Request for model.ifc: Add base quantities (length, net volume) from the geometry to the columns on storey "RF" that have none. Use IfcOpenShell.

First a look at what the model holds.

```python
import ifcopenshell
import ifcopenshell.util.element
import ifcopenshell.util.unit

model = ifcopenshell.open("model.ifc")
print(model.schema)
for unit_type in ("LENGTHUNIT", "AREAUNIT", "VOLUMEUNIT"):
    print(unit_type, ifcopenshell.util.unit.calculate_unit_scale(model, unit_type))
storey = next(s for s in model.by_type("IfcBuildingStorey") if s.Name == "RF")
columns = [e for e in ifcopenshell.util.element.get_decomposition(storey) if e.is_a("IfcColumn")]
for e in sorted(columns, key=lambda e: e.id()):
    print(e.id(), e.is_a(), e.Name, list(ifcopenshell.util.element.get_psets(e, qtos_only=True)), sep=" | ")
```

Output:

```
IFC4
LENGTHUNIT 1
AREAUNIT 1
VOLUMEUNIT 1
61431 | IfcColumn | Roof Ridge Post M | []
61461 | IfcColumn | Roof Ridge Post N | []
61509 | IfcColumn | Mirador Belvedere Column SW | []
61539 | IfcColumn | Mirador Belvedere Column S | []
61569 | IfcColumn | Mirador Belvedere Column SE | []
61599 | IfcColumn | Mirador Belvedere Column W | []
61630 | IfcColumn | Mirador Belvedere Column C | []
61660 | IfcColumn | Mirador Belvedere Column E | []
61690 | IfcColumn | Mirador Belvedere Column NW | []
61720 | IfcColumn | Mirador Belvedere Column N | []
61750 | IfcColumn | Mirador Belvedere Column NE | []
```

```python
import ifcopenshell
import ifcopenshell.api.pset
import ifcopenshell.geom
import ifcopenshell.util.element
import ifcopenshell.util.shape
import ifcopenshell.util.unit

model = ifcopenshell.open("model.ifc")
unit_scale = ifcopenshell.util.unit.calculate_unit_scale(model)
volume_scale = ifcopenshell.util.unit.calculate_unit_scale(model, "VOLUMEUNIT")
settings = ifcopenshell.geom.settings()

storey = next(s for s in model.by_type("IfcBuildingStorey") if s.Name == "RF")
columns = [e for e in ifcopenshell.util.element.get_decomposition(storey) if e.is_a("IfcColumn")]

for e in sorted(columns, key=lambda e: e.id()):
    if ifcopenshell.util.element.get_psets(e, qtos_only=True, should_inherit=False):
        continue
    # Geometry comes back in metres, in the element's own axes.
    shape = ifcopenshell.geom.create_shape(settings, e)
    values = {
        "Length": ifcopenshell.util.shape.get_z(shape.geometry) / unit_scale,
        "NetVolume": ifcopenshell.util.shape.get_volume(shape.geometry) / volume_scale,
    }
    qto = ifcopenshell.api.pset.add_qto(model, product=e, name="Qto_ColumnBaseQuantities")
    ifcopenshell.api.pset.edit_qto(model, qto=qto, properties=values)
    print(e.id(), {k: round(v, 3) for k, v in values.items()})

model.write("model-out.ifc")
```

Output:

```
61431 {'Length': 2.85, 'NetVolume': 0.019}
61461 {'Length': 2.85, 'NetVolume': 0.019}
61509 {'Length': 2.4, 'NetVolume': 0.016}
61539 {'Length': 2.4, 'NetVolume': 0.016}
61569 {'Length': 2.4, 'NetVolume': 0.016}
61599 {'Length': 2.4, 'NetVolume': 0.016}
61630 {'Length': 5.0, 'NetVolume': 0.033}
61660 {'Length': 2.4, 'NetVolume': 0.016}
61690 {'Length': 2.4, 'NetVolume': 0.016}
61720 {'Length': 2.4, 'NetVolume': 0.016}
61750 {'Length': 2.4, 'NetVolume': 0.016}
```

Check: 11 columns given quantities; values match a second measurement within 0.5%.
